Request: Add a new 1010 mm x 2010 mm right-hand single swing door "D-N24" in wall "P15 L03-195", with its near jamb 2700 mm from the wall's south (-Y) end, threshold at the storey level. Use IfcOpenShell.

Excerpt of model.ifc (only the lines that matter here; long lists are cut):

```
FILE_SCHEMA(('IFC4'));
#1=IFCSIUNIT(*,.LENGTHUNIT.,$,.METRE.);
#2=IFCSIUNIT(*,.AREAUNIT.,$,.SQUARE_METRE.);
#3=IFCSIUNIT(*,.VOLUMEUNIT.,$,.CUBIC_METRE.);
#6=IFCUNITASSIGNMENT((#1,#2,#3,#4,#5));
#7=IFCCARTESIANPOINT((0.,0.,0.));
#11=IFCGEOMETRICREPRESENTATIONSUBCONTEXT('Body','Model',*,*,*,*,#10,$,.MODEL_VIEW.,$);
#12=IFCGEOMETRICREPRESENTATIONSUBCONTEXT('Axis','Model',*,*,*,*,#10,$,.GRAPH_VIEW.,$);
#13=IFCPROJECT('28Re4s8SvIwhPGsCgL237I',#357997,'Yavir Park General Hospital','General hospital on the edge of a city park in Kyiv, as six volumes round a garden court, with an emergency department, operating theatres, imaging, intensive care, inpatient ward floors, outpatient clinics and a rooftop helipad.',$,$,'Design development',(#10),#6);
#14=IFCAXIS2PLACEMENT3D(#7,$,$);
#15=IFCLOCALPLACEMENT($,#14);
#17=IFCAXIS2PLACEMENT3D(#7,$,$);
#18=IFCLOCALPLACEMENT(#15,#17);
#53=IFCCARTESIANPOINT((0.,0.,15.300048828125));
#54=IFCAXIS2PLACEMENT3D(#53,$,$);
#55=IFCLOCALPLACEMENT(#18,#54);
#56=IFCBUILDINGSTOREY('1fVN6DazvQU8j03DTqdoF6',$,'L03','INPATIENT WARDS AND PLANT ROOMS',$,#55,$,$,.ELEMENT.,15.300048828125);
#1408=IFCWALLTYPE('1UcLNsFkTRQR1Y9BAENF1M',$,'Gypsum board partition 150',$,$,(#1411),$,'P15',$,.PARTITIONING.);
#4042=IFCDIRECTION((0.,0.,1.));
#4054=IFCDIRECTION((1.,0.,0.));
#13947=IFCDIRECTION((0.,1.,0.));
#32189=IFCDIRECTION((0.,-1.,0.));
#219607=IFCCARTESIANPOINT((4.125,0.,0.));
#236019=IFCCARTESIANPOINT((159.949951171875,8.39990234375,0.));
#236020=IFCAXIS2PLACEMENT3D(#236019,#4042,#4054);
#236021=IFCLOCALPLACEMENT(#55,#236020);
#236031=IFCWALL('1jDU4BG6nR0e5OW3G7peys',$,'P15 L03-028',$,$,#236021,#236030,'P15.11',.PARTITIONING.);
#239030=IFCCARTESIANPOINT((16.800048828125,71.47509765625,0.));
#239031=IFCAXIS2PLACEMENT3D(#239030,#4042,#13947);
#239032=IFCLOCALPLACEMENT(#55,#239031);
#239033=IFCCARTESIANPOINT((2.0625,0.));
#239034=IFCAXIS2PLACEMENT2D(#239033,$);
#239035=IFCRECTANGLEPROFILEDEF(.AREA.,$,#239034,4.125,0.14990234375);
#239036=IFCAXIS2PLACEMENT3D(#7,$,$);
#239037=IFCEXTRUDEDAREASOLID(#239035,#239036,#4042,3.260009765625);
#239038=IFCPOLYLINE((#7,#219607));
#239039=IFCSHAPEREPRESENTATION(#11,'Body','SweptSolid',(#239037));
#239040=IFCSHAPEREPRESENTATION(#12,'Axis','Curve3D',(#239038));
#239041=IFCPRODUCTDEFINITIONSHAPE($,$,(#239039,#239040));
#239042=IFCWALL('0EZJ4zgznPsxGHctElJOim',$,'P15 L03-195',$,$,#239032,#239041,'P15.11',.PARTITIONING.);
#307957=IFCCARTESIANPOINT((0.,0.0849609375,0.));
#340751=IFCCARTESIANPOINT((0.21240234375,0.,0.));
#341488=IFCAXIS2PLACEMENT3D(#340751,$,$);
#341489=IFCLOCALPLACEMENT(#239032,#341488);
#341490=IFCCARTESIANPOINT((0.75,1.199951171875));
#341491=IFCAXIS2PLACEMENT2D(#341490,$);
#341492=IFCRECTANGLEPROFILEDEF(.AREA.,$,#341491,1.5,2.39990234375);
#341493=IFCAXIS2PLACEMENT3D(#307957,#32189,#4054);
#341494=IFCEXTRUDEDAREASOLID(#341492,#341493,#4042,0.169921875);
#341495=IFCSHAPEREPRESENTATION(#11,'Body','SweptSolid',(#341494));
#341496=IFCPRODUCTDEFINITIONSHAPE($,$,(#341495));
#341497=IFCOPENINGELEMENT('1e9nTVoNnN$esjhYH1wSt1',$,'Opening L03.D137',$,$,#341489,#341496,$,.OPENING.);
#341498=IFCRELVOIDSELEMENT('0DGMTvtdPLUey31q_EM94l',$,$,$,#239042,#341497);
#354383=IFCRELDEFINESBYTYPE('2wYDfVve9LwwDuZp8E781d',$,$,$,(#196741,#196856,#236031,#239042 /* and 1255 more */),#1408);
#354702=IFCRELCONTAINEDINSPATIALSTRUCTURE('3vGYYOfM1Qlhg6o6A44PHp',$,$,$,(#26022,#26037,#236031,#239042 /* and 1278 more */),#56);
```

```python
import numpy as np
import ifcopenshell
import ifcopenshell.api.feature
import ifcopenshell.api.geometry
import ifcopenshell.api.root
import ifcopenshell.api.spatial
import ifcopenshell.geom
import ifcopenshell.util.element
import ifcopenshell.util.placement
import ifcopenshell.util.representation
import ifcopenshell.util.shape
import ifcopenshell.util.unit

model = ifcopenshell.open("model.ifc")
unit_scale = ifcopenshell.util.unit.calculate_unit_scale(model)
settings = ifcopenshell.geom.settings()


def volume(element):
    """Net volume in cubic metres, openings subtracted."""
    shape = ifcopenshell.geom.create_shape(settings, element)
    return ifcopenshell.util.shape.get_volume(shape.geometry)


wall = model.by_guid("0EZJ4zgznPsxGHctElJOim")
storey = ifcopenshell.util.element.get_container(wall, ifc_class="IfcBuildingStorey")
context = ifcopenshell.util.representation.get_context(model, "Model", "Body", "MODEL_VIEW")
before = volume(wall)

width, height, from_end, sill = 1.01, 2.01, 2.7, 0.0  # metres

# The wall runs along its own X axis, and the end named is its -X end.
wall_shape = ifcopenshell.geom.create_shape(settings, wall)
x, y, z = ifcopenshell.util.shape.get_vertices(wall_shape.geometry).T
start = x.min() + from_end
face, thickness = float(y.min()), float(y.max() - y.min())
wall_matrix = ifcopenshell.util.placement.get_local_placement(wall.ObjectPlacement)
level = ifcopenshell.util.placement.get_local_placement(storey.ObjectPlacement)[2, 3]


def in_wall(x, y):
    """Placement at x, y metres in the wall's axes, at sill height."""
    matrix = wall_matrix.copy()
    matrix[:, 3] = wall_matrix @ np.array([x / unit_scale, y / unit_scale, 0.0, 1.0])
    matrix[2, 3] = level + sill / unit_scale
    return matrix


# Opening: a box that overshoots both wall faces by 50 mm.
opening = ifcopenshell.api.root.create_entity(model, ifc_class="IfcOpeningElement", predefined_type="OPENING")
box = ifcopenshell.api.geometry.add_wall_representation(
    model, context=context, length=width, height=height, thickness=thickness + 0.1
)
ifcopenshell.api.geometry.assign_representation(model, product=opening, representation=box)
ifcopenshell.api.geometry.edit_object_placement(model, product=opening, matrix=in_wall(start, face - 0.05), is_si=False)
ifcopenshell.api.feature.add_feature(model, feature=opening, element=wall)

door = ifcopenshell.api.root.create_entity(model, ifc_class="IfcDoor", name="D-N24", predefined_type="DOOR")
door.OverallWidth, door.OverallHeight = width / unit_scale, height / unit_scale
door.OperationType = "SINGLE_SWING_RIGHT"
body = ifcopenshell.api.geometry.add_door_representation(
    model,
    context=context,
    overall_width=door.OverallWidth,
    overall_height=door.OverallHeight,
    operation_type="SINGLE_SWING_RIGHT",
    lining_properties={"LiningDepth": thickness / unit_scale, "ThresholdDepth": thickness / unit_scale},
)
ifcopenshell.api.geometry.assign_representation(model, product=door, representation=body)
ifcopenshell.api.spatial.assign_container(model, products=[door], relating_structure=storey)
ifcopenshell.api.feature.add_filling(model, opening=opening, element=door)

# The lining spans the wall, so the door starts at the wall face.
ifcopenshell.api.geometry.edit_object_placement(model, product=door, matrix=in_wall(start, face), is_si=False)

after = volume(wall)

print(f"wall volume {before:.3f} -> {after:.3f} m3")

model.write("model_updated.ifc")
```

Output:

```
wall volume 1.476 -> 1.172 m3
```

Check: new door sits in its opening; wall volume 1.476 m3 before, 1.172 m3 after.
